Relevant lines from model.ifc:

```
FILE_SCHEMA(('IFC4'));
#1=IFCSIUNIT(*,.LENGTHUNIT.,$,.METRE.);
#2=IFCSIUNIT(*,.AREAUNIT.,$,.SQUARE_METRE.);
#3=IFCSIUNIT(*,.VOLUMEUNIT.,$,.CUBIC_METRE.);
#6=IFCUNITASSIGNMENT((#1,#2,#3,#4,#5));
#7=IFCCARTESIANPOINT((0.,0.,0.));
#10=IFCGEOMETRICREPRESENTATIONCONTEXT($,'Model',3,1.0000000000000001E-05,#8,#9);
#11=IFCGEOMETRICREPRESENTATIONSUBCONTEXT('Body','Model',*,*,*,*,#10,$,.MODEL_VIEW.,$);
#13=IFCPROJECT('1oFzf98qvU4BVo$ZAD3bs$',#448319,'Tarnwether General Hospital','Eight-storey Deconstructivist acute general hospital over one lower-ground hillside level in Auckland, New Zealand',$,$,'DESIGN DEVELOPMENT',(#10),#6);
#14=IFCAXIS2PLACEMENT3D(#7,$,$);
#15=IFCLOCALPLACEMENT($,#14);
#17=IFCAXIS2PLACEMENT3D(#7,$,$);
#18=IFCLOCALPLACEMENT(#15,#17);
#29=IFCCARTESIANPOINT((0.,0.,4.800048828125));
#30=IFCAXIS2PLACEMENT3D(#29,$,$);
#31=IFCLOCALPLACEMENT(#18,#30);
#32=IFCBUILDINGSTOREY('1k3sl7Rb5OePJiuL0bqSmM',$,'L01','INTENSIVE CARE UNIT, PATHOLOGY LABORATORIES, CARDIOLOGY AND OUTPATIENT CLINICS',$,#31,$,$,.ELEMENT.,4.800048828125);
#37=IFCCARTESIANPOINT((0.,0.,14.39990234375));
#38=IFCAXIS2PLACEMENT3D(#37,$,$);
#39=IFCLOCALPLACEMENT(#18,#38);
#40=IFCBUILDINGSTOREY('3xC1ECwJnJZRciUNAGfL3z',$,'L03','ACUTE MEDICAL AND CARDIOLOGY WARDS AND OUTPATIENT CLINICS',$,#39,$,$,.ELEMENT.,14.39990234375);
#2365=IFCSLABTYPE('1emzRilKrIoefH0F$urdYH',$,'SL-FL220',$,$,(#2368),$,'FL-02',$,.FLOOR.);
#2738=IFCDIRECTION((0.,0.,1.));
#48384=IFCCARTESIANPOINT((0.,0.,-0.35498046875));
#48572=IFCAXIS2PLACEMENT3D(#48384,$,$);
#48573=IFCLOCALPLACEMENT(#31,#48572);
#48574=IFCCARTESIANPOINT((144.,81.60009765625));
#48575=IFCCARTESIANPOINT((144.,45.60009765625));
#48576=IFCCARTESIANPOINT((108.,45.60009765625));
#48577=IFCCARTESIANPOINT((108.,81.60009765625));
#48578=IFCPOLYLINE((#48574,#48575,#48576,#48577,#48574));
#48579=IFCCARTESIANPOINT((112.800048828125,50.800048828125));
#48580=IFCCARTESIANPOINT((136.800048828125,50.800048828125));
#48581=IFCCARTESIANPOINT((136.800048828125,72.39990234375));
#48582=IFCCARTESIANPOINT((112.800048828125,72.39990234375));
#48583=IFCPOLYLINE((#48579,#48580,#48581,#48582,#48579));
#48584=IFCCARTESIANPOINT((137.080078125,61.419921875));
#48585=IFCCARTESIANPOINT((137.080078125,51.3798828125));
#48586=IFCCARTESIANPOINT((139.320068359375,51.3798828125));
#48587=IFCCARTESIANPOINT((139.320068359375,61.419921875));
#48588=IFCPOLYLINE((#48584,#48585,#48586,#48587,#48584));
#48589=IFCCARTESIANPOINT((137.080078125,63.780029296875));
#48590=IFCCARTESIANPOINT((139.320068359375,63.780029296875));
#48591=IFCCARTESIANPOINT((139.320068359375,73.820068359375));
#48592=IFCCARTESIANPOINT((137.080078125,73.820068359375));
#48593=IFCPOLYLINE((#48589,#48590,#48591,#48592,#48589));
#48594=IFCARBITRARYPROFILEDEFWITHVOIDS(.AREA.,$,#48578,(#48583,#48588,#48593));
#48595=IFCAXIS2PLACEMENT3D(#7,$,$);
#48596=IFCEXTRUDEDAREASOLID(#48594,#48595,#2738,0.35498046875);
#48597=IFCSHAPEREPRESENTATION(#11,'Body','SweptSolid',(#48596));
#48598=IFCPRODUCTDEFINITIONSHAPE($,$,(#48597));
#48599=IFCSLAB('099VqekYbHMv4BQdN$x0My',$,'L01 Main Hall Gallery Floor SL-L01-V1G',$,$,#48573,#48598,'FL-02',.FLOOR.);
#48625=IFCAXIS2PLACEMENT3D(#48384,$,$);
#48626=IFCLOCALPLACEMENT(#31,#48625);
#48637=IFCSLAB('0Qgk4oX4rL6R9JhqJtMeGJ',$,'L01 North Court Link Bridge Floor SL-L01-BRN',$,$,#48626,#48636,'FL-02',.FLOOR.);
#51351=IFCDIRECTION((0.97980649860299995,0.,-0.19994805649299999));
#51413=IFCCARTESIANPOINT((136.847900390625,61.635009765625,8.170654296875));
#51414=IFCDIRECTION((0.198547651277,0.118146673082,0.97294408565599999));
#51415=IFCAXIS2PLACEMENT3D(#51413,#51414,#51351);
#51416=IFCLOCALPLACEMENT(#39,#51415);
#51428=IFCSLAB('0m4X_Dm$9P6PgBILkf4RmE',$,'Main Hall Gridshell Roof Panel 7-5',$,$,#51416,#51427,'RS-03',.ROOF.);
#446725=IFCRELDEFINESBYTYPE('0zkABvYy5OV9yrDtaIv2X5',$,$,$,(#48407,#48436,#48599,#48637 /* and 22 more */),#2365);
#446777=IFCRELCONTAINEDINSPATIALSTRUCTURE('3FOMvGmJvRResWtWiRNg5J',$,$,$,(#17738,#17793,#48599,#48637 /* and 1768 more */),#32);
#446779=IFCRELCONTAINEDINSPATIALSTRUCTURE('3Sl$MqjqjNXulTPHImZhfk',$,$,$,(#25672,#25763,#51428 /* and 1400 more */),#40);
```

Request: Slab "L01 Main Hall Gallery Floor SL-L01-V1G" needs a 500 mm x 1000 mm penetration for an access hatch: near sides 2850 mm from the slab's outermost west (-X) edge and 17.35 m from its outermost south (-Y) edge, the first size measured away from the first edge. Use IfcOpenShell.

```python
import numpy as np
import ifcopenshell
import ifcopenshell.api.feature
import ifcopenshell.api.geometry
import ifcopenshell.api.root
import ifcopenshell.geom
import ifcopenshell.util.placement
import ifcopenshell.util.representation
import ifcopenshell.util.shape
import ifcopenshell.util.unit

model = ifcopenshell.open("model.ifc")
unit_scale = ifcopenshell.util.unit.calculate_unit_scale(model)
settings = ifcopenshell.geom.settings()


def volume(element):
    """Net volume in cubic metres, openings subtracted."""
    shape = ifcopenshell.geom.create_shape(settings, element)
    return ifcopenshell.util.shape.get_volume(shape.geometry)


slab = model.by_guid("099VqekYbHMv4BQdN$x0My")
before = volume(slab)

# Extent in the slab's own axes, in metres. The edges named are its -X and -Y sides.
slab_shape = ifcopenshell.geom.create_shape(settings, slab)
vertices = ifcopenshell.util.shape.get_vertices(slab_shape.geometry)
x_min, y_min, bottom = vertices.min(axis=0)
top = vertices[:, 2].max()

opening = ifcopenshell.api.root.create_entity(model, ifc_class="IfcOpeningElement", name="Access hatch opening", predefined_type="OPENING")
context = ifcopenshell.util.representation.get_context(model, "Model", "Body", "MODEL_VIEW")
width, depth = 0.5, 1
outline = [(0.0, 0.0), (width, 0.0), (width, depth), (0.0, depth), (0.0, 0.0)]
# Overshoot both faces by 50 mm so the cut is clean.
shape = ifcopenshell.api.geometry.add_slab_representation(
    model, context=context, depth=top - bottom + 0.1, polyline=outline
)
ifcopenshell.api.geometry.assign_representation(model, product=opening, representation=shape)

matrix = ifcopenshell.util.placement.get_local_placement(slab.ObjectPlacement)
matrix[:, 3] = matrix @ np.append(np.array([x_min + 2.85, y_min + 17.35, bottom - 0.05]) / unit_scale, 1.0)
ifcopenshell.api.geometry.edit_object_placement(model, product=opening, matrix=matrix, is_si=False)
ifcopenshell.api.feature.add_feature(model, feature=opening, element=slab)

after = volume(slab)

print(f"slab volume {before:.3f} -> {after:.3f} m3")

model.write("model_updated.ifc")
```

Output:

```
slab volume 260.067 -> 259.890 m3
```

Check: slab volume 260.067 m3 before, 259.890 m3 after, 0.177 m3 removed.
